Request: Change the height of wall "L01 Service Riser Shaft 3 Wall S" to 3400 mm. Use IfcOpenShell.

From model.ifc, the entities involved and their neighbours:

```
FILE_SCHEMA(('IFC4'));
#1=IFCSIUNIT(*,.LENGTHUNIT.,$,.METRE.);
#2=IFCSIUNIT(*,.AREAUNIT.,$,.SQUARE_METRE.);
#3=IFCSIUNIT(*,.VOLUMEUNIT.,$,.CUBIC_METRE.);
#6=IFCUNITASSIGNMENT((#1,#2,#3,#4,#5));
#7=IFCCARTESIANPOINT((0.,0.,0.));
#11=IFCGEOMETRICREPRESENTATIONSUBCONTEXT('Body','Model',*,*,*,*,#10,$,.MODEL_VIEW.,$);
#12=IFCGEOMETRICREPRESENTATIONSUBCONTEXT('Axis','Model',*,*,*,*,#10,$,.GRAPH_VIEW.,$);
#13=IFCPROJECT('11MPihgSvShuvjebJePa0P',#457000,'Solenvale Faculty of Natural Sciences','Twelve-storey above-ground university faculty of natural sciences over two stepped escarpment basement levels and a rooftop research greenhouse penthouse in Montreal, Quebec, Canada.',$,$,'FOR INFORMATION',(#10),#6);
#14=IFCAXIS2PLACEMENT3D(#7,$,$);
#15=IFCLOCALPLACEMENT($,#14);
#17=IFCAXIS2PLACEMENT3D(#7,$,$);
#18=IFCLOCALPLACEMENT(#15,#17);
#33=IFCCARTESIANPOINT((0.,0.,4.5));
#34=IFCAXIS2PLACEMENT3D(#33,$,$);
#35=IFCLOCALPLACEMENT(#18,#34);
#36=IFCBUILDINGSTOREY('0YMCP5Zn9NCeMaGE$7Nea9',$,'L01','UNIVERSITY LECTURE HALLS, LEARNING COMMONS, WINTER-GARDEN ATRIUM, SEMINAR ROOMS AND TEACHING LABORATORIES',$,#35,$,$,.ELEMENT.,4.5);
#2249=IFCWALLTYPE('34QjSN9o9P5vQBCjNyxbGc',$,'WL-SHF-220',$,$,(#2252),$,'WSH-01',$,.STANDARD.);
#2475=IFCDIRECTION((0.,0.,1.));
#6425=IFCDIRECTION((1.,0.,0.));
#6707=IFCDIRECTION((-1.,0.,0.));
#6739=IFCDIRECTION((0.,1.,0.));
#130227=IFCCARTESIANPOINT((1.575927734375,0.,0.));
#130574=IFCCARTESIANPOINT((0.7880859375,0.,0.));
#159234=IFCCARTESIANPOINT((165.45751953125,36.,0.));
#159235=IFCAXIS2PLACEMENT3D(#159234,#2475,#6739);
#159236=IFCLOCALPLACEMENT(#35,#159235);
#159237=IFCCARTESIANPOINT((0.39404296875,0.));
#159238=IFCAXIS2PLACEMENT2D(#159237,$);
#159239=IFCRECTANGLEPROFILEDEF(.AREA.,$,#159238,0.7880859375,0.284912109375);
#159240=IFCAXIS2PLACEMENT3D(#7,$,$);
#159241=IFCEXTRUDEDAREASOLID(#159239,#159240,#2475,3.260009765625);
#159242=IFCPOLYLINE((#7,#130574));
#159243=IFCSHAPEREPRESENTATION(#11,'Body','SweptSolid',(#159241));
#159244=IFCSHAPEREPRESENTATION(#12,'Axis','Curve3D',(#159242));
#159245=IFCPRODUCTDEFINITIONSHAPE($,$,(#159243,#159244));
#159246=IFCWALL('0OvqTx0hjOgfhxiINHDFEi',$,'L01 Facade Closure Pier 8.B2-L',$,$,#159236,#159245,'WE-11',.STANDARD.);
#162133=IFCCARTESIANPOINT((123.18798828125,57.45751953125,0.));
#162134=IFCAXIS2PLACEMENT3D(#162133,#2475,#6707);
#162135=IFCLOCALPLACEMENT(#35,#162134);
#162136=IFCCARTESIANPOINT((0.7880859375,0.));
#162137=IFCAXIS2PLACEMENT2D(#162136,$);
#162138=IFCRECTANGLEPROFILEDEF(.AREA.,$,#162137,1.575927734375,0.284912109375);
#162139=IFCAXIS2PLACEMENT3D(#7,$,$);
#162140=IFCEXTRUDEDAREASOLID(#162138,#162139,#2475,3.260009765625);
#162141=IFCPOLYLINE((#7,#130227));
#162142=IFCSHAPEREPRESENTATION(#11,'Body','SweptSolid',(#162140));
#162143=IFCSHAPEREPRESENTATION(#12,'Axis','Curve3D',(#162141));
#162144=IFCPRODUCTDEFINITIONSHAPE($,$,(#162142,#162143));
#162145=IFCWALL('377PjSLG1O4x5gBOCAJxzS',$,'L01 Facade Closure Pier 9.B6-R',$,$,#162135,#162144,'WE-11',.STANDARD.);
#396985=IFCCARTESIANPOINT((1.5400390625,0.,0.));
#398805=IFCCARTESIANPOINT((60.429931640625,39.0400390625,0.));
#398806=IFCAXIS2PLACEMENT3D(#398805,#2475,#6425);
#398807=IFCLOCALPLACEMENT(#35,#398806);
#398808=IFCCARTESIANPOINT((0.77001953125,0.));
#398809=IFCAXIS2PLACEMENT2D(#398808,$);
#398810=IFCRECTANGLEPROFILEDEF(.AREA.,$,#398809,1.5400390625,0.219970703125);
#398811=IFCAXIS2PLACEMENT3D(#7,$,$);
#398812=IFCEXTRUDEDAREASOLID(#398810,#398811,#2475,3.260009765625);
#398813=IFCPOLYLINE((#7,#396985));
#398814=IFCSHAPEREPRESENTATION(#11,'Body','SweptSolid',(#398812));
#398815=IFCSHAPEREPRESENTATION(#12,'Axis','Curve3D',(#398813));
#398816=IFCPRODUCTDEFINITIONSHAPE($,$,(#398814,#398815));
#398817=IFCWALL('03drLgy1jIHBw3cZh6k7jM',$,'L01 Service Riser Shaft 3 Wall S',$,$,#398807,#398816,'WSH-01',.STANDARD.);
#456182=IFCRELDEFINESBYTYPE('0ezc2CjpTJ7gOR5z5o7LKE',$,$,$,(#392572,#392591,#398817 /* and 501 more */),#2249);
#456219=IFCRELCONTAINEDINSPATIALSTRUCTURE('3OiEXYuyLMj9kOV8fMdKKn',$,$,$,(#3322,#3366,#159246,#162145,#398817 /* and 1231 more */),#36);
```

```python
import ifcopenshell
import ifcopenshell.geom
import ifcopenshell.util.representation
import ifcopenshell.util.shape
import ifcopenshell.util.unit

model = ifcopenshell.open("model.ifc")
unit_scale = ifcopenshell.util.unit.calculate_unit_scale(model)
settings = ifcopenshell.geom.settings()


def volume(element):
    """Net volume in cubic metres, openings subtracted."""
    shape = ifcopenshell.geom.create_shape(settings, element)
    return ifcopenshell.util.shape.get_volume(shape.geometry)


wall = model.by_guid("03drLgy1jIHBw3cZh6k7jM")
before = volume(wall)

body = ifcopenshell.util.representation.get_representation(wall, "Model", "Body")
solid = body.Items[0]
old_height = solid.Depth
solid.Depth = 3.4 / unit_scale
after = volume(wall)

print(f"height {old_height:g} -> {solid.Depth:g}, volume {before:.3f} -> {after:.3f} m3")

model.write("model_edited.ifc")
```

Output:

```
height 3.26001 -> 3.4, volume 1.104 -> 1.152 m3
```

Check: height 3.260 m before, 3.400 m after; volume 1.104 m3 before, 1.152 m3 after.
